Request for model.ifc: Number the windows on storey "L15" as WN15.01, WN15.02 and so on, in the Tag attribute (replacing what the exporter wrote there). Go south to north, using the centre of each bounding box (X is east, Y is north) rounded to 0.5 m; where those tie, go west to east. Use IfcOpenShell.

First a look at what the model holds.

```python
import ifcopenshell
import ifcopenshell.util.element
import ifcopenshell.util.placement

model = ifcopenshell.open("model.ifc")
print(model.schema)
storey = next(s for s in model.by_type("IfcBuildingStorey") if s.Name == "L15")
windows = [e for e in ifcopenshell.util.element.get_decomposition(storey) if e.is_a("IfcWindow")]
for e in sorted(windows, key=lambda e: e.id()):
    origin = ifcopenshell.util.placement.get_local_placement(e.ObjectPlacement)[:3, 3]
    print(e.id(), e.Tag, e.Name, origin.round(2) + 0.0, sep=" | ")
```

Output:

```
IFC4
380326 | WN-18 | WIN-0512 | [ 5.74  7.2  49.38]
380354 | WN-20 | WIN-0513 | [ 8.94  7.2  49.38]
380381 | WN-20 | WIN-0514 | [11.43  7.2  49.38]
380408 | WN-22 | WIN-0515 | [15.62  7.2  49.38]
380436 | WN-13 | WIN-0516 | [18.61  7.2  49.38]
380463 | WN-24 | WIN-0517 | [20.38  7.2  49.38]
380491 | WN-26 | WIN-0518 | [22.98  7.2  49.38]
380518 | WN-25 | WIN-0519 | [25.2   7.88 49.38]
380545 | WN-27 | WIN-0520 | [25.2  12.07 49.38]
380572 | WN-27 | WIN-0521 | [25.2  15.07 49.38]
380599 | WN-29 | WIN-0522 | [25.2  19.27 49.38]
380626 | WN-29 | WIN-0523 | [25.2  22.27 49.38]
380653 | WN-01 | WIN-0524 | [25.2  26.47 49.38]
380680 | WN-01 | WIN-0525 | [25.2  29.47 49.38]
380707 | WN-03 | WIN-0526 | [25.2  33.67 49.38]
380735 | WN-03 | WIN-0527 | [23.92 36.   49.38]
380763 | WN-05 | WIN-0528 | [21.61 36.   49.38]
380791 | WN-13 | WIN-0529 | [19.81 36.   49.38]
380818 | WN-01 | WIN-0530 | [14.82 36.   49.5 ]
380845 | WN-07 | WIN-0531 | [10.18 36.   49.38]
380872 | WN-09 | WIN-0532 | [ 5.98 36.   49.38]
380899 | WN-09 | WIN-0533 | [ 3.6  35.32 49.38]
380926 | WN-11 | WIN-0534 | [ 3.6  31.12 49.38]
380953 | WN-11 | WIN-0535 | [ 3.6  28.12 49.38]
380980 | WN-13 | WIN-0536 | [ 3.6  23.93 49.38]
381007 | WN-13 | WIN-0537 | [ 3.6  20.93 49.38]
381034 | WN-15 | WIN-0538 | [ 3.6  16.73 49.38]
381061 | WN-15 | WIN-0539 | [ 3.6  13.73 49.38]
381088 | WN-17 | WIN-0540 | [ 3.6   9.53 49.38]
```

```python
import ifcopenshell
import ifcopenshell.geom
import ifcopenshell.util.element
import ifcopenshell.util.shape

model = ifcopenshell.open("model.ifc")
settings = ifcopenshell.geom.settings()
settings.set("use-world-coords", True)


def centre(element):
    shape = ifcopenshell.geom.create_shape(settings, element)
    return ifcopenshell.util.shape.get_bbox_centroid(shape.geometry)


storey = next(s for s in model.by_type("IfcBuildingStorey") if s.Name == "L15")
windows = [e for e in ifcopenshell.util.element.get_decomposition(storey) if e.is_a("IfcWindow")]

# Insertion points can sit at a corner or the storey origin, so sort by the geometry (in metres).
centres = {e: centre(e) for e in windows}
windows.sort(key=lambda e: (round(centres[e][1] / 0.5), centres[e][0]))

for i, e in enumerate(windows, start=1):
    number = f"WN15.{i:02d}"
    e.Tag = number
    print(e.id(), number)

model.write("model_updated.ifc")
```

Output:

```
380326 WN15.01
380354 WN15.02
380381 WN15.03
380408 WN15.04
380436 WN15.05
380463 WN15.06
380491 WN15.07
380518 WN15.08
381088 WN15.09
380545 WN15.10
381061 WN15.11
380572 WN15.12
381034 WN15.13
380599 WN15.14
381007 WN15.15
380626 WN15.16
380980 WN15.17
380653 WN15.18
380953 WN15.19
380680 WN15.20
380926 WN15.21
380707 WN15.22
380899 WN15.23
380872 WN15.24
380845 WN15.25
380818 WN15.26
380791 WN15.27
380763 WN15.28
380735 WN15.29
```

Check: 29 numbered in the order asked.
